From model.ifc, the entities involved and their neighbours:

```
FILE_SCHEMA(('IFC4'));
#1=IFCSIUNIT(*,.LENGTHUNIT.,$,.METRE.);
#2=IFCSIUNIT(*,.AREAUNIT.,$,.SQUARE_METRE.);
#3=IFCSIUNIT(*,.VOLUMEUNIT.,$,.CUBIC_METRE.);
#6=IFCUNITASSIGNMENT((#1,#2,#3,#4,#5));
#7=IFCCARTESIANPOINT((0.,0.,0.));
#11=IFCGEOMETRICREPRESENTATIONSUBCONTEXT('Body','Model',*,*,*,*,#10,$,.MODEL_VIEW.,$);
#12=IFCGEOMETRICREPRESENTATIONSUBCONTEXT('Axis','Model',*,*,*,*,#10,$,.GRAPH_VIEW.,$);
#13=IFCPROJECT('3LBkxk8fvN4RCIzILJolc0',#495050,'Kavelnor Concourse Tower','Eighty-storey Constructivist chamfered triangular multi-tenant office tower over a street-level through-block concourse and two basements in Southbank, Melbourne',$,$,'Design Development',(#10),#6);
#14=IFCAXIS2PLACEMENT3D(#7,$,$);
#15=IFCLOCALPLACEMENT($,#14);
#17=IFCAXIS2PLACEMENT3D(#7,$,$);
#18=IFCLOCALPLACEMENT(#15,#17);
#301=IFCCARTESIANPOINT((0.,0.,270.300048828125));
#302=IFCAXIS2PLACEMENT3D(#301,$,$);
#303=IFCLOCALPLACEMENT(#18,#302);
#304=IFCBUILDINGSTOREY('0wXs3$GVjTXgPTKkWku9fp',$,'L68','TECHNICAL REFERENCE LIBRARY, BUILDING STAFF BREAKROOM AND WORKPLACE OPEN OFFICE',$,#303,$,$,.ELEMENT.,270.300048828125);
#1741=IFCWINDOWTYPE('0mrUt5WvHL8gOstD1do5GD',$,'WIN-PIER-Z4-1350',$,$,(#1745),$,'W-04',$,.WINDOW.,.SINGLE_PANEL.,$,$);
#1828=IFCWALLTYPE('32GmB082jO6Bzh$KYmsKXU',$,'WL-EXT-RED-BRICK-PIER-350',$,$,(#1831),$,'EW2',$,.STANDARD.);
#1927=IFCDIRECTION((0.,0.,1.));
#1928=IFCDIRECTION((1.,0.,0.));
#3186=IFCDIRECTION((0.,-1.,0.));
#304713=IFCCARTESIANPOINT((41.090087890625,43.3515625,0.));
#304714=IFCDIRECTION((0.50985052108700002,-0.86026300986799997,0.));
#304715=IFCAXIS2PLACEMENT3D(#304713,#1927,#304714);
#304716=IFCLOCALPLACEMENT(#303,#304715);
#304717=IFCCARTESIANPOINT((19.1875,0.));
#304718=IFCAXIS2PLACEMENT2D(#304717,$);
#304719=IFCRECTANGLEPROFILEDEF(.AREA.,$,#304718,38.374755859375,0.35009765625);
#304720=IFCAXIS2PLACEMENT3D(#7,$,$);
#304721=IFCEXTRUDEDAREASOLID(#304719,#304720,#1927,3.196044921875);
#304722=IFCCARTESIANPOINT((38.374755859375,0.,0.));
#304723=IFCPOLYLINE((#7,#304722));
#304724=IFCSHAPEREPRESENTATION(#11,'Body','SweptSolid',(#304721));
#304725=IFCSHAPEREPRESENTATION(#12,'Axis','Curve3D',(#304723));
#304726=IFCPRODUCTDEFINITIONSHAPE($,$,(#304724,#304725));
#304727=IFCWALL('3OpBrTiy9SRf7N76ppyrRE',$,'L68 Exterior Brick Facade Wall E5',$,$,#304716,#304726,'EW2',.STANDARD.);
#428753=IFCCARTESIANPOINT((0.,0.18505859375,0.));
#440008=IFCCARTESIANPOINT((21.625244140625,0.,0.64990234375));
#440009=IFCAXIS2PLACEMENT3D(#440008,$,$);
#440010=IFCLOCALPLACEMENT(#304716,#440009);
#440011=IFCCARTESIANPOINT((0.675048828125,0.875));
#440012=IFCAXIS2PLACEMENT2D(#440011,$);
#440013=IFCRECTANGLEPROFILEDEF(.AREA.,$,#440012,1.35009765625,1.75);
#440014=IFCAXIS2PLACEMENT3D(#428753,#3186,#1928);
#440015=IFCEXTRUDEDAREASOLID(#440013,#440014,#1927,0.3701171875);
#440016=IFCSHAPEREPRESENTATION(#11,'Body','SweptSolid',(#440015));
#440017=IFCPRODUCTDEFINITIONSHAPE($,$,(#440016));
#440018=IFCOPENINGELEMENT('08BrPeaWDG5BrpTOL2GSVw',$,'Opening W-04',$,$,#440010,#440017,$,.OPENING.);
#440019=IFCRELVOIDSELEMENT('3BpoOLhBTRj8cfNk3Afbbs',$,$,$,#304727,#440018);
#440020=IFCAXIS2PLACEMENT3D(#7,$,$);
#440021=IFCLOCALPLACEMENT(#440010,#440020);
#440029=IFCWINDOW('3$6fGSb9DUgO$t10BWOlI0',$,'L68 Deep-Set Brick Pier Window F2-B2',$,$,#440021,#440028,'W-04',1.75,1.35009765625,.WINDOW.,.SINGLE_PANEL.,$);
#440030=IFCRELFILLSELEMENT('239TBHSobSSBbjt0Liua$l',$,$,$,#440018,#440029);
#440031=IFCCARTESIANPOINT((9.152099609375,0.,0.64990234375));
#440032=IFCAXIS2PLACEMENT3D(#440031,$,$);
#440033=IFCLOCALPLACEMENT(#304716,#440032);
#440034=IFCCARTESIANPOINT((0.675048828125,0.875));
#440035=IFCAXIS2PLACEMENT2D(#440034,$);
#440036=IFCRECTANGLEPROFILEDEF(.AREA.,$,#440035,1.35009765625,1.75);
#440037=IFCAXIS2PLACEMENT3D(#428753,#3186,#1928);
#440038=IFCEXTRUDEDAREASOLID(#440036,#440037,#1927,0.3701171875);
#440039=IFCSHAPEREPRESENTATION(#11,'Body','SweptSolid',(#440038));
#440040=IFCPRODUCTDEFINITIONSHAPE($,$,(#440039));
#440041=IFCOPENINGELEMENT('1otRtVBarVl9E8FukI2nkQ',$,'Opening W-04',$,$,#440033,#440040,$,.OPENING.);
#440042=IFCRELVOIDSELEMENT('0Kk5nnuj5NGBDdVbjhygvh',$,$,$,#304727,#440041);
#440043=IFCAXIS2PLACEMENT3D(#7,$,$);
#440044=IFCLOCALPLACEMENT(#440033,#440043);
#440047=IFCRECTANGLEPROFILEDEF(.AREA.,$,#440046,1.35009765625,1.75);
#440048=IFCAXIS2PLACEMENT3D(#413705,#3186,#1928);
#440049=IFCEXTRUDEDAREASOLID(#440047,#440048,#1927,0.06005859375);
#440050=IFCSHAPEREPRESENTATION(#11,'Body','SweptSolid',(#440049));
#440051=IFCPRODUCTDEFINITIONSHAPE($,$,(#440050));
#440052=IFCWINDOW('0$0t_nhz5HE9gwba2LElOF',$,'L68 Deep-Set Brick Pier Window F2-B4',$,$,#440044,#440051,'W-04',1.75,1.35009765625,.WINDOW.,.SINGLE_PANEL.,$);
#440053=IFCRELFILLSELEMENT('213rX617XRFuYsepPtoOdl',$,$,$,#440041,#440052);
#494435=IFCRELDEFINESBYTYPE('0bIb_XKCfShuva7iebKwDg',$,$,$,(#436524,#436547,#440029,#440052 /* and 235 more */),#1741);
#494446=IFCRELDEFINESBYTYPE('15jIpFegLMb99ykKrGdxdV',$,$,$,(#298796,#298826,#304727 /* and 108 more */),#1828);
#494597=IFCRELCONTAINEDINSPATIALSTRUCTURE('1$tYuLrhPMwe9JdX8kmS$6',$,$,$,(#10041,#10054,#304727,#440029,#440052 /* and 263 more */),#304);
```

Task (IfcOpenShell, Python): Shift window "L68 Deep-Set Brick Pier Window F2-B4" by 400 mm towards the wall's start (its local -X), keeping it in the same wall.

```python
import ifcopenshell
import ifcopenshell.api.geometry
import ifcopenshell.util.placement

model = ifcopenshell.open("model.ifc")

window = model.by_id(440052)
opening = window.FillsVoids[0].RelatingOpeningElement
wall = opening.VoidsElements[0].RelatingBuildingElement

wall_matrix = ifcopenshell.util.placement.get_local_placement(wall.ObjectPlacement)
shift = wall_matrix[:3, 0] * -0.4
before = ifcopenshell.util.placement.get_local_placement(window.ObjectPlacement)[:3, 3].copy()

# The window is placed relative to its opening, so it follows when the opening moves.
matrix = ifcopenshell.util.placement.get_local_placement(opening.ObjectPlacement)
matrix[:3, 3] += shift
ifcopenshell.api.geometry.edit_object_placement(
    model, product=opening, matrix=matrix, is_si=False, should_transform_children=True
)

after = ifcopenshell.util.placement.get_local_placement(window.ObjectPlacement)[:3, 3]
print("window moved by", (after - before).round(3) + 0.0)

model.write("model-out.ifc")
```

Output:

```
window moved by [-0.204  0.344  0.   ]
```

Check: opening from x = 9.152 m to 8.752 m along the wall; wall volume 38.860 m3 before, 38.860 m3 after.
